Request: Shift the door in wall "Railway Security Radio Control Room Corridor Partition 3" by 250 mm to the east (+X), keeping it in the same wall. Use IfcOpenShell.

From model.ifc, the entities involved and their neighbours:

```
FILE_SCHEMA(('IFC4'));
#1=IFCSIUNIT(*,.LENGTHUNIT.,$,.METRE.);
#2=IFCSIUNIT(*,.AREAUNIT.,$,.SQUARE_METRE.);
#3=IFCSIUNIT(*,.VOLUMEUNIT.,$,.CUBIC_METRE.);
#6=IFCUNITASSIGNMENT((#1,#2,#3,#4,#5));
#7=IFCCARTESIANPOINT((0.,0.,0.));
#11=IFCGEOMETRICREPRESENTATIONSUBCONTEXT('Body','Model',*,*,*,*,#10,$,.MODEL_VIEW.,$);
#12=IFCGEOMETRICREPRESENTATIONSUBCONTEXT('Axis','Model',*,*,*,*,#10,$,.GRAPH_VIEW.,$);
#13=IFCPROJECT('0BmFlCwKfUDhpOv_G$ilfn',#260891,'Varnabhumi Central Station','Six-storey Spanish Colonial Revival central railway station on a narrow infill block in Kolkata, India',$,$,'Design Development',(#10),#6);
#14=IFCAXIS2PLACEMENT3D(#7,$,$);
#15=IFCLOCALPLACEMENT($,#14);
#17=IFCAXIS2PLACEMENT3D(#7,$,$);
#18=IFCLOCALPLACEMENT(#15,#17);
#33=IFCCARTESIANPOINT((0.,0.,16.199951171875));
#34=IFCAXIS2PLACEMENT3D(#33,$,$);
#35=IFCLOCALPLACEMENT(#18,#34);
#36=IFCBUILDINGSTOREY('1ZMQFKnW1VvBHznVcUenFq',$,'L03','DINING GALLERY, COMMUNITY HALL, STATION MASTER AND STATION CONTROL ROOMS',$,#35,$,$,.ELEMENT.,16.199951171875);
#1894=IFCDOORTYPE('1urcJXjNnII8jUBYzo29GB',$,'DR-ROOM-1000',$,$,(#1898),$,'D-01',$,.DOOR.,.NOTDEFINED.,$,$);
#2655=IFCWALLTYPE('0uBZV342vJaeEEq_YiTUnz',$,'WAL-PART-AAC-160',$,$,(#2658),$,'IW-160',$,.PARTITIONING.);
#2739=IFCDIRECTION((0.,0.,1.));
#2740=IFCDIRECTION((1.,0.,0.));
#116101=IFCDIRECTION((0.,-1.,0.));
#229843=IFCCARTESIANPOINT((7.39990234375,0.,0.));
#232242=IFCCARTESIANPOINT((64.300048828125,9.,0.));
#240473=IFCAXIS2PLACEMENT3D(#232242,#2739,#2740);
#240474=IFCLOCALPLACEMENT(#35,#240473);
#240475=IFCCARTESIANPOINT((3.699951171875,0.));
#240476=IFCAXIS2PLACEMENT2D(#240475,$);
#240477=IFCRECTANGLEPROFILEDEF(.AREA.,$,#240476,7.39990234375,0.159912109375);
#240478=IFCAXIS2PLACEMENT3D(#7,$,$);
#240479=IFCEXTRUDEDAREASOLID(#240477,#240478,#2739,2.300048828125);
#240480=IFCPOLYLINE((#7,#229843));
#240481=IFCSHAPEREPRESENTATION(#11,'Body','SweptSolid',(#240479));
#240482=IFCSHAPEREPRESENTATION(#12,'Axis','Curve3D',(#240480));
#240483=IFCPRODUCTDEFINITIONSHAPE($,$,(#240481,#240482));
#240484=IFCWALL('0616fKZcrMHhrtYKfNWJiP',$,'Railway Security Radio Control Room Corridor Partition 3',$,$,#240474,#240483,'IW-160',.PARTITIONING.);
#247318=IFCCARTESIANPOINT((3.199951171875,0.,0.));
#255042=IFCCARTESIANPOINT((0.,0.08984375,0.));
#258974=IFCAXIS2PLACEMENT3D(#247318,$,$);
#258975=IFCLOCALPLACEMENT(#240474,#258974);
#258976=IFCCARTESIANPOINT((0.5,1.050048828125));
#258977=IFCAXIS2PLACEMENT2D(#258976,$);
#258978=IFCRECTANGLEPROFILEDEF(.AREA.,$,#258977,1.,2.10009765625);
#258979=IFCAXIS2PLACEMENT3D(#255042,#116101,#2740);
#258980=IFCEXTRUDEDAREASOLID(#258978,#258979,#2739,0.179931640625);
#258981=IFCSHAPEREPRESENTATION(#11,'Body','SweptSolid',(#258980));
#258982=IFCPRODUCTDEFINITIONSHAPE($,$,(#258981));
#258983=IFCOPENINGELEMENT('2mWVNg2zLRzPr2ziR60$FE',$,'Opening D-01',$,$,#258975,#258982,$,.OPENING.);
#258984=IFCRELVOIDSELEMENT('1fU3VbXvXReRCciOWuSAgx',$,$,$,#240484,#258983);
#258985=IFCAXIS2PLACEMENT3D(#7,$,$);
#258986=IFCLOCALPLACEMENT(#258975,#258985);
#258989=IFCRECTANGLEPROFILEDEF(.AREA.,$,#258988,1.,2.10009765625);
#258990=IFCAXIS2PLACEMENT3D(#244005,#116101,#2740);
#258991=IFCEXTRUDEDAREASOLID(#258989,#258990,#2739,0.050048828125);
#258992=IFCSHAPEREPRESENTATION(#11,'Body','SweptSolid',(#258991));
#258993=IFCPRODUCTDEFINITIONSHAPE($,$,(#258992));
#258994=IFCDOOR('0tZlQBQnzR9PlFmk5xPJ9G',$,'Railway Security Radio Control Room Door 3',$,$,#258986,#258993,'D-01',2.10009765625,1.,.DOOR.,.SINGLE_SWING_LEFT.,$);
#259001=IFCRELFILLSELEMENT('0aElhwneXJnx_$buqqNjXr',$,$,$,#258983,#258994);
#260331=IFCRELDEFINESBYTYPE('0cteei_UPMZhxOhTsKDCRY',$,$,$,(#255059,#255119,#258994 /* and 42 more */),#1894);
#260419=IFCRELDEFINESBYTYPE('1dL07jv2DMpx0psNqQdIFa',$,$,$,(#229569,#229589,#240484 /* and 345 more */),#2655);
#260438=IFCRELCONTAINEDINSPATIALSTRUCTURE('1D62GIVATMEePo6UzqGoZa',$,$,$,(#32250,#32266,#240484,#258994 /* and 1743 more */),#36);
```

```python
import ifcopenshell
import ifcopenshell.api.geometry
import ifcopenshell.util.placement
import ifcopenshell.util.unit

model = ifcopenshell.open("model.ifc")
unit_scale = ifcopenshell.util.unit.calculate_unit_scale(model)

door = model.by_guid("0tZlQBQnzR9PlFmk5xPJ9G")
opening = door.FillsVoids[0].RelatingOpeningElement
wall = opening.VoidsElements[0].RelatingBuildingElement

wall_matrix = ifcopenshell.util.placement.get_local_placement(wall.ObjectPlacement)
shift = wall_matrix[:3, 0] * 0.25 / unit_scale
before = ifcopenshell.util.placement.get_local_placement(door.ObjectPlacement)[:3, 3].copy()

# The door is placed relative to its opening, so it follows when the opening moves.
matrix = ifcopenshell.util.placement.get_local_placement(opening.ObjectPlacement)
matrix[:3, 3] += shift
ifcopenshell.api.geometry.edit_object_placement(
    model, product=opening, matrix=matrix, is_si=False, should_transform_children=True
)

after = ifcopenshell.util.placement.get_local_placement(door.ObjectPlacement)[:3, 3]
print("door moved by", (after - before).round(3) + 0.0)

model.write("model_updated.ifc")
```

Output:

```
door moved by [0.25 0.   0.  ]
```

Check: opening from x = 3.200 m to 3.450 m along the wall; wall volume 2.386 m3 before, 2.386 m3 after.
